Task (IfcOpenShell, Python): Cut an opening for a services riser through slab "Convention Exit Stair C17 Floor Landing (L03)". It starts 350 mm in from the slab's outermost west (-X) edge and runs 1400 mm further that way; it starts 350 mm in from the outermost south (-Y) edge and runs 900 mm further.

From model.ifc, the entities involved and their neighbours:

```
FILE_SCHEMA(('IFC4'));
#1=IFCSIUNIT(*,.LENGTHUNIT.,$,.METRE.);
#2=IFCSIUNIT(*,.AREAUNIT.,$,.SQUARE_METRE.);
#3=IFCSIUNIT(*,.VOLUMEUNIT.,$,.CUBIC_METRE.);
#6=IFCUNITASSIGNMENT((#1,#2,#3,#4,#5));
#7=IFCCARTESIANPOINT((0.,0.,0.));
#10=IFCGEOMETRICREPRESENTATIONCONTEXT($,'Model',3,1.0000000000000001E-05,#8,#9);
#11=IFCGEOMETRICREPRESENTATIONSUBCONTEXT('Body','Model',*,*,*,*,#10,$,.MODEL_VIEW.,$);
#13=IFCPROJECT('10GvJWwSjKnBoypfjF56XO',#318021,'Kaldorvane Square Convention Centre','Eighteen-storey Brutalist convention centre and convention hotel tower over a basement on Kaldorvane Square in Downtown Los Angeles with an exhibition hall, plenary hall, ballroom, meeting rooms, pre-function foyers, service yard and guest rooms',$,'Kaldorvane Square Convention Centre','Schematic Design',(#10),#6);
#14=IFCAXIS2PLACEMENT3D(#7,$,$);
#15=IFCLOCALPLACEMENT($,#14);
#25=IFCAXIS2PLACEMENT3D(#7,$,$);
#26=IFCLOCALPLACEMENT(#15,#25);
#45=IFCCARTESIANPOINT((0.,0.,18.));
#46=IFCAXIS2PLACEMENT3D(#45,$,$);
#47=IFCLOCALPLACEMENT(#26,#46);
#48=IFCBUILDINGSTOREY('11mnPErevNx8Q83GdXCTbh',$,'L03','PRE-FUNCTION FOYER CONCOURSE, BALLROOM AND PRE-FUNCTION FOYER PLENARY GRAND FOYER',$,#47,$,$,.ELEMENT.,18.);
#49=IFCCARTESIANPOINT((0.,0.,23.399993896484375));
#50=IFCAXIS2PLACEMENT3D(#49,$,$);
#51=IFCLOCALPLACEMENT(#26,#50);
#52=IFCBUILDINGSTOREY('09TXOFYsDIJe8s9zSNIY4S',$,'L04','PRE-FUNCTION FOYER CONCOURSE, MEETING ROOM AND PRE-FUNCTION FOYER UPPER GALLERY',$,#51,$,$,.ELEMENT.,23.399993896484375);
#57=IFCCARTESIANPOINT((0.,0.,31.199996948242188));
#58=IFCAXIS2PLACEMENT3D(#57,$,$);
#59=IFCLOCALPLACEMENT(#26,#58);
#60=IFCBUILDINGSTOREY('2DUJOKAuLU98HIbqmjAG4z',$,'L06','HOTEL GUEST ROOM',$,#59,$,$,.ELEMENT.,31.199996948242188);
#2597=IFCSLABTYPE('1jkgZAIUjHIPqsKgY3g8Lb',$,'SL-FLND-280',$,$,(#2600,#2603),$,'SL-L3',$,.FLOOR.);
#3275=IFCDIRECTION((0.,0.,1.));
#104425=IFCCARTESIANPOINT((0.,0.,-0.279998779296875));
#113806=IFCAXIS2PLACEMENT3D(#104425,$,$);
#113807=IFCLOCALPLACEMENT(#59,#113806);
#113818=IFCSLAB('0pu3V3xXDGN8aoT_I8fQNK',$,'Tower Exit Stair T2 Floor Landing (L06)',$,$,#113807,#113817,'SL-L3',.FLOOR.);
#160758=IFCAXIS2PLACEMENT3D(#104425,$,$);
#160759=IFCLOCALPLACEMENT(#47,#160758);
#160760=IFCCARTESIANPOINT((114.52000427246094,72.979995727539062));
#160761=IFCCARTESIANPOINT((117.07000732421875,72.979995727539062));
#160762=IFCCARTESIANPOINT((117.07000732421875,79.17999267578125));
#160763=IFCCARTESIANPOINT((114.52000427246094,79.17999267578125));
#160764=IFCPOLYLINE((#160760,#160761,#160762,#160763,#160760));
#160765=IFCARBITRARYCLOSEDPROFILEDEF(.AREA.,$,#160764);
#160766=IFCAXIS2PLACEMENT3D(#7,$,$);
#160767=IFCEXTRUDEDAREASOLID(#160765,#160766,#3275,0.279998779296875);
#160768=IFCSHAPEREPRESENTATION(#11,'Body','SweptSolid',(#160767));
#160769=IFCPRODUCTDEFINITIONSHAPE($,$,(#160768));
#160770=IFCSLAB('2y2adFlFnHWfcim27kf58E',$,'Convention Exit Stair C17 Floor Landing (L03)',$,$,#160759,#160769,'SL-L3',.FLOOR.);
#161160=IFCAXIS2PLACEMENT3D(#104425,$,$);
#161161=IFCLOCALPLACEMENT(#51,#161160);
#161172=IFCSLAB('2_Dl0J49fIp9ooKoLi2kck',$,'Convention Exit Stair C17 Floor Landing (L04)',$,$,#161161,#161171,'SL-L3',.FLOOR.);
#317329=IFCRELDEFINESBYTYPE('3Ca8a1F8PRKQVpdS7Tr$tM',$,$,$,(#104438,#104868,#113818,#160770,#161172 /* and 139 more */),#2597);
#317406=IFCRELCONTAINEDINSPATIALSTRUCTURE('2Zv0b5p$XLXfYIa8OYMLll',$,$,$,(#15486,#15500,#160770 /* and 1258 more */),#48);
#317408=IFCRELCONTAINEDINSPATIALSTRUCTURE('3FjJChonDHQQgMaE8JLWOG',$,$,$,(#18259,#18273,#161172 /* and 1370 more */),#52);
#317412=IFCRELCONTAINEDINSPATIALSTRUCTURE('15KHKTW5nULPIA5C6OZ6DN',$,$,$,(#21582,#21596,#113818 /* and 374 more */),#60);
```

```python
import numpy as np
import ifcopenshell
import ifcopenshell.api.feature
import ifcopenshell.api.geometry
import ifcopenshell.api.root
import ifcopenshell.geom
import ifcopenshell.util.placement
import ifcopenshell.util.representation
import ifcopenshell.util.shape
import ifcopenshell.util.unit

model = ifcopenshell.open("model.ifc")
unit_scale = ifcopenshell.util.unit.calculate_unit_scale(model)
settings = ifcopenshell.geom.settings()


def volume(element):
    """Net volume in cubic metres, openings subtracted."""
    shape = ifcopenshell.geom.create_shape(settings, element)
    return ifcopenshell.util.shape.get_volume(shape.geometry)


slab = model.by_guid("2y2adFlFnHWfcim27kf58E")
before = volume(slab)

# Extent in the slab's own axes, in metres. The edges named are its -X and -Y sides.
slab_shape = ifcopenshell.geom.create_shape(settings, slab)
vertices = ifcopenshell.util.shape.get_vertices(slab_shape.geometry)
x_min, y_min, bottom = vertices.min(axis=0)
top = vertices[:, 2].max()

opening = ifcopenshell.api.root.create_entity(model, ifc_class="IfcOpeningElement", name="Services riser opening", predefined_type="OPENING")
context = ifcopenshell.util.representation.get_context(model, "Model", "Body", "MODEL_VIEW")
width, depth = 1.4, 0.9
outline = [(0.0, 0.0), (width, 0.0), (width, depth), (0.0, depth), (0.0, 0.0)]
# Overshoot both faces by 50 mm so the cut is clean.
shape = ifcopenshell.api.geometry.add_slab_representation(
    model, context=context, depth=top - bottom + 0.1, polyline=outline
)
ifcopenshell.api.geometry.assign_representation(model, product=opening, representation=shape)

matrix = ifcopenshell.util.placement.get_local_placement(slab.ObjectPlacement)
matrix[:, 3] = matrix @ np.append(np.array([x_min + 0.35, y_min + 0.35, bottom - 0.05]) / unit_scale, 1.0)
ifcopenshell.api.geometry.edit_object_placement(model, product=opening, matrix=matrix, is_si=False)
ifcopenshell.api.feature.add_feature(model, feature=opening, element=slab)

after = volume(slab)

print(f"slab volume {before:.3f} -> {after:.3f} m3")

model.write("model_edited.ifc")
```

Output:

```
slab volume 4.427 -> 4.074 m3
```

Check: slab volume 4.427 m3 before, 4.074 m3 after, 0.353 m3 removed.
